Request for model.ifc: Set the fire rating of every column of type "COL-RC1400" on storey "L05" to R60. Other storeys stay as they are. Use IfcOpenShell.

First a look at what the model holds.

```python
import ifcopenshell
import ifcopenshell.util.element

model = ifcopenshell.open("model.ifc")
print(model.schema)
storey = next(s for s in model.by_type("IfcBuildingStorey") if s.Name == "L05")
columns = [e for e in ifcopenshell.util.element.get_decomposition(storey) if e.is_a("IfcColumn")]
seen = {}
for e in columns:
    element_type = ifcopenshell.util.element.get_type(e)
    key = (element_type.Name if element_type != e and element_type else None, ifcopenshell.util.element.get_pset(e, "Pset_ColumnCommon", "FireRating"))
    seen[key] = seen.get(key, 0) + 1
for (name, value), count in sorted(seen.items(), key=str):
    print(count, "x", name, "|", value)
```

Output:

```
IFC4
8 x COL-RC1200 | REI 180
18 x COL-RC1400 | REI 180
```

```python
import ifcopenshell
import ifcopenshell.api.pset
import ifcopenshell.util.element

model = ifcopenshell.open("model.ifc")

storey = next(s for s in model.by_type("IfcBuildingStorey") if s.Name == "L05")
columns = [e for e in ifcopenshell.util.element.get_decomposition(storey) if e.is_a("IfcColumn")]

count = 0
for e in columns:
    element_type = ifcopenshell.util.element.get_type(e)
    if element_type in (None, e) or element_type.Name != "COL-RC1400":
        continue
    # add_pset returns the element's existing set when there is one.
    pset = ifcopenshell.api.pset.add_pset(model, product=e, name="Pset_ColumnCommon")
    ifcopenshell.api.pset.edit_pset(model, pset=pset, properties={"FireRating": "R60"})
    count += 1

print(count, "columns updated")

model.write("model_updated.ifc")
```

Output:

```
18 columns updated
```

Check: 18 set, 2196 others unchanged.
